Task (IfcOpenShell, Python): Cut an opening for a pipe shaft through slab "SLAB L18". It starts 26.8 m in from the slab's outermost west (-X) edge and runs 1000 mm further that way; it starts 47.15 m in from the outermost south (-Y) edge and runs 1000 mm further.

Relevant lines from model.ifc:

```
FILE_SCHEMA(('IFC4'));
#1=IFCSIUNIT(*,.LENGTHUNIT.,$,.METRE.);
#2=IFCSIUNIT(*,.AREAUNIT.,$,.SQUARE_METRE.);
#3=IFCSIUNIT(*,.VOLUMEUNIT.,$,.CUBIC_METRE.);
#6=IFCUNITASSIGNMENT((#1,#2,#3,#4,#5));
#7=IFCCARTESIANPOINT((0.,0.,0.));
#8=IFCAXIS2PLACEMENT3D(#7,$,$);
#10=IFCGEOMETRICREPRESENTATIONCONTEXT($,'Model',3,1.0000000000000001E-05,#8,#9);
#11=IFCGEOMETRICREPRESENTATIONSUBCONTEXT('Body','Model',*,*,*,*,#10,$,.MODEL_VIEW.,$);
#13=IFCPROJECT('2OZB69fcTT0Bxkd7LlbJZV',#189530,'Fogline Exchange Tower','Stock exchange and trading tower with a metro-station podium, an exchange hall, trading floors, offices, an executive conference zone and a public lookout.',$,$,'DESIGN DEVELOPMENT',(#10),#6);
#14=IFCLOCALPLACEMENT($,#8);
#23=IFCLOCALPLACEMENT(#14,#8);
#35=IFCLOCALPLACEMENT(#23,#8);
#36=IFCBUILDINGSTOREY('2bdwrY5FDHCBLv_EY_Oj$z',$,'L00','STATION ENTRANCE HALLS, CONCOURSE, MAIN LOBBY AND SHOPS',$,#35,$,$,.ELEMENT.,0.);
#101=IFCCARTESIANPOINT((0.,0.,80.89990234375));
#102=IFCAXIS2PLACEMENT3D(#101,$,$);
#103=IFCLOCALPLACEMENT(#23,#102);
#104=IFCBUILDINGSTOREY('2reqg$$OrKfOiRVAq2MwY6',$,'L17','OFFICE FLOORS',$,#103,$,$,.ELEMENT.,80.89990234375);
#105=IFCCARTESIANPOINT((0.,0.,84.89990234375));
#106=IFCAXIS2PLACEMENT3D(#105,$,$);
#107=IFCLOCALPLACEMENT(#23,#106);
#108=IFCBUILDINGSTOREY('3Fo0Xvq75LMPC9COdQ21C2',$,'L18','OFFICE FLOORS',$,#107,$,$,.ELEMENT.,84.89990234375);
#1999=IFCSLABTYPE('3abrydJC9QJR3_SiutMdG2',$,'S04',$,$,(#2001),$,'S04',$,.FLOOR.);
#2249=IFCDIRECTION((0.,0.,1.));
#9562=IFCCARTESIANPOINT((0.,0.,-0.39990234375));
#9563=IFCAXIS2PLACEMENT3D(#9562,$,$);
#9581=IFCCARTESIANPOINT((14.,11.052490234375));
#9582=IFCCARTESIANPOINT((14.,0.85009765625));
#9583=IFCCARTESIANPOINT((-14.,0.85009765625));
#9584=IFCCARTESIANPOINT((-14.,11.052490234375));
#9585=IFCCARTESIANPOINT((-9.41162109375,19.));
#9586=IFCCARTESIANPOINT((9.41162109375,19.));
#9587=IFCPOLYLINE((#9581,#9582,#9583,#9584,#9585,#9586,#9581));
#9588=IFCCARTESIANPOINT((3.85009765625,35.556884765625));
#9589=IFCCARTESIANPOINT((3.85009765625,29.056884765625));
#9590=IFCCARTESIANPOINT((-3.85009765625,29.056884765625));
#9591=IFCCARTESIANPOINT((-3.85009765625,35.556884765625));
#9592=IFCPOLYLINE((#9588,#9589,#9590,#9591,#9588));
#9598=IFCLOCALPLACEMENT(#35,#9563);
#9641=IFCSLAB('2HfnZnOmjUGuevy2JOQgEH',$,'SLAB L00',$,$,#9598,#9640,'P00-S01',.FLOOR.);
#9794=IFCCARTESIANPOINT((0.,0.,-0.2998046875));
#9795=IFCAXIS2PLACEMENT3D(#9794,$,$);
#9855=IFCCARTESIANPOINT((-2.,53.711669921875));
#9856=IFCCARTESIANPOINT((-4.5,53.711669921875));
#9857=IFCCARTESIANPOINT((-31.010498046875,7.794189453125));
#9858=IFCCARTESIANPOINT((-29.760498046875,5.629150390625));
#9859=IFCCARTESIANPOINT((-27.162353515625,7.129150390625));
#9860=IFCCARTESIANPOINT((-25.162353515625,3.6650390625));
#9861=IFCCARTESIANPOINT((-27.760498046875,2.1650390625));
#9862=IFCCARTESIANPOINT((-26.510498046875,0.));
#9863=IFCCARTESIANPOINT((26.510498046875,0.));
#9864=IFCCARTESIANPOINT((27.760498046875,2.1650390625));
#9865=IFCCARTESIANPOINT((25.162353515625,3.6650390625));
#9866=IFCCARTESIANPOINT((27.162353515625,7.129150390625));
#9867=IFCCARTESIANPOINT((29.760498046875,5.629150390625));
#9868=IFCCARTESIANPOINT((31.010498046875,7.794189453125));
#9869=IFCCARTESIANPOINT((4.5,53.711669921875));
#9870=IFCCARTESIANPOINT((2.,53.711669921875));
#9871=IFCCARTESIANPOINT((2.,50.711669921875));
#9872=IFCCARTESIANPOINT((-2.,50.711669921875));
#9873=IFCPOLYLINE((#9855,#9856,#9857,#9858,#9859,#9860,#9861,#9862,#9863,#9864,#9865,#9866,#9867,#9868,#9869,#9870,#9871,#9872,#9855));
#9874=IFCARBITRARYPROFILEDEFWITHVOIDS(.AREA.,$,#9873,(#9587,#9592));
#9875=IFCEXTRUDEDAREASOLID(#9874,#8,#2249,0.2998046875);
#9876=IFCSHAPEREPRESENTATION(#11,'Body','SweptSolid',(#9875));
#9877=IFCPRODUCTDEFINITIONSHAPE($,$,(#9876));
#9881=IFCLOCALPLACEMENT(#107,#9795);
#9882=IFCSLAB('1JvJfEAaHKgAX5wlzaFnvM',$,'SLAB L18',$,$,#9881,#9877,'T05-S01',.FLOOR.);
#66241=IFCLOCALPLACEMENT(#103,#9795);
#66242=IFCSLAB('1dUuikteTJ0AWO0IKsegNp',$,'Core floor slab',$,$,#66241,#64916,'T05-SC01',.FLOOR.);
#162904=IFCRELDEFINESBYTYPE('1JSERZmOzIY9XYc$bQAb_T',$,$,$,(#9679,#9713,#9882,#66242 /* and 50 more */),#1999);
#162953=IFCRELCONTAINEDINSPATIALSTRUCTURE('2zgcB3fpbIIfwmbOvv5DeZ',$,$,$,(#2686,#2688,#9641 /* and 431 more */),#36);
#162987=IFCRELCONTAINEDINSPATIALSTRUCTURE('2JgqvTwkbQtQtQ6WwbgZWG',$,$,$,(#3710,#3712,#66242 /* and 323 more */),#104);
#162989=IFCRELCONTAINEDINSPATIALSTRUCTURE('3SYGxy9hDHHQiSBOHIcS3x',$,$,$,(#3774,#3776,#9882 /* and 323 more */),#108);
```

```python
import numpy as np
import ifcopenshell
import ifcopenshell.api.feature
import ifcopenshell.api.geometry
import ifcopenshell.api.root
import ifcopenshell.geom
import ifcopenshell.util.placement
import ifcopenshell.util.representation
import ifcopenshell.util.shape
import ifcopenshell.util.unit

model = ifcopenshell.open("model.ifc")
unit_scale = ifcopenshell.util.unit.calculate_unit_scale(model)
settings = ifcopenshell.geom.settings()


def volume(element):
    """Net volume in cubic metres, openings subtracted."""
    shape = ifcopenshell.geom.create_shape(settings, element)
    return ifcopenshell.util.shape.get_volume(shape.geometry)


slab = model.by_id(9882)
before = volume(slab)

# Extent in the slab's own axes, in metres. The edges named are its -X and -Y sides.
slab_shape = ifcopenshell.geom.create_shape(settings, slab)
vertices = ifcopenshell.util.shape.get_vertices(slab_shape.geometry)
x_min, y_min, bottom = vertices.min(axis=0)
top = vertices[:, 2].max()

opening = ifcopenshell.api.root.create_entity(model, ifc_class="IfcOpeningElement", name="Pipe shaft opening", predefined_type="OPENING")
context = ifcopenshell.util.representation.get_context(model, "Model", "Body", "MODEL_VIEW")
width, depth = 1, 1
outline = [(0.0, 0.0), (width, 0.0), (width, depth), (0.0, depth), (0.0, 0.0)]
# Overshoot both faces by 50 mm so the cut is clean.
shape = ifcopenshell.api.geometry.add_slab_representation(
    model, context=context, depth=top - bottom + 0.1, polyline=outline
)
ifcopenshell.api.geometry.assign_representation(model, product=opening, representation=shape)

matrix = ifcopenshell.util.placement.get_local_placement(slab.ObjectPlacement)
matrix[:, 3] = matrix @ np.append(np.array([x_min + 26.8, y_min + 47.15, bottom - 0.05]) / unit_scale, 1.0)
ifcopenshell.api.geometry.edit_object_placement(model, product=opening, matrix=matrix, is_si=False)
ifcopenshell.api.feature.add_feature(model, feature=opening, element=slab)

after = volume(slab)

print(f"slab volume {before:.3f} -> {after:.3f} m3")

model.write("model_rev.ifc")
```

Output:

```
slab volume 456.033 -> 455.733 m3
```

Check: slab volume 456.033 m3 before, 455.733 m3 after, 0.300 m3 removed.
